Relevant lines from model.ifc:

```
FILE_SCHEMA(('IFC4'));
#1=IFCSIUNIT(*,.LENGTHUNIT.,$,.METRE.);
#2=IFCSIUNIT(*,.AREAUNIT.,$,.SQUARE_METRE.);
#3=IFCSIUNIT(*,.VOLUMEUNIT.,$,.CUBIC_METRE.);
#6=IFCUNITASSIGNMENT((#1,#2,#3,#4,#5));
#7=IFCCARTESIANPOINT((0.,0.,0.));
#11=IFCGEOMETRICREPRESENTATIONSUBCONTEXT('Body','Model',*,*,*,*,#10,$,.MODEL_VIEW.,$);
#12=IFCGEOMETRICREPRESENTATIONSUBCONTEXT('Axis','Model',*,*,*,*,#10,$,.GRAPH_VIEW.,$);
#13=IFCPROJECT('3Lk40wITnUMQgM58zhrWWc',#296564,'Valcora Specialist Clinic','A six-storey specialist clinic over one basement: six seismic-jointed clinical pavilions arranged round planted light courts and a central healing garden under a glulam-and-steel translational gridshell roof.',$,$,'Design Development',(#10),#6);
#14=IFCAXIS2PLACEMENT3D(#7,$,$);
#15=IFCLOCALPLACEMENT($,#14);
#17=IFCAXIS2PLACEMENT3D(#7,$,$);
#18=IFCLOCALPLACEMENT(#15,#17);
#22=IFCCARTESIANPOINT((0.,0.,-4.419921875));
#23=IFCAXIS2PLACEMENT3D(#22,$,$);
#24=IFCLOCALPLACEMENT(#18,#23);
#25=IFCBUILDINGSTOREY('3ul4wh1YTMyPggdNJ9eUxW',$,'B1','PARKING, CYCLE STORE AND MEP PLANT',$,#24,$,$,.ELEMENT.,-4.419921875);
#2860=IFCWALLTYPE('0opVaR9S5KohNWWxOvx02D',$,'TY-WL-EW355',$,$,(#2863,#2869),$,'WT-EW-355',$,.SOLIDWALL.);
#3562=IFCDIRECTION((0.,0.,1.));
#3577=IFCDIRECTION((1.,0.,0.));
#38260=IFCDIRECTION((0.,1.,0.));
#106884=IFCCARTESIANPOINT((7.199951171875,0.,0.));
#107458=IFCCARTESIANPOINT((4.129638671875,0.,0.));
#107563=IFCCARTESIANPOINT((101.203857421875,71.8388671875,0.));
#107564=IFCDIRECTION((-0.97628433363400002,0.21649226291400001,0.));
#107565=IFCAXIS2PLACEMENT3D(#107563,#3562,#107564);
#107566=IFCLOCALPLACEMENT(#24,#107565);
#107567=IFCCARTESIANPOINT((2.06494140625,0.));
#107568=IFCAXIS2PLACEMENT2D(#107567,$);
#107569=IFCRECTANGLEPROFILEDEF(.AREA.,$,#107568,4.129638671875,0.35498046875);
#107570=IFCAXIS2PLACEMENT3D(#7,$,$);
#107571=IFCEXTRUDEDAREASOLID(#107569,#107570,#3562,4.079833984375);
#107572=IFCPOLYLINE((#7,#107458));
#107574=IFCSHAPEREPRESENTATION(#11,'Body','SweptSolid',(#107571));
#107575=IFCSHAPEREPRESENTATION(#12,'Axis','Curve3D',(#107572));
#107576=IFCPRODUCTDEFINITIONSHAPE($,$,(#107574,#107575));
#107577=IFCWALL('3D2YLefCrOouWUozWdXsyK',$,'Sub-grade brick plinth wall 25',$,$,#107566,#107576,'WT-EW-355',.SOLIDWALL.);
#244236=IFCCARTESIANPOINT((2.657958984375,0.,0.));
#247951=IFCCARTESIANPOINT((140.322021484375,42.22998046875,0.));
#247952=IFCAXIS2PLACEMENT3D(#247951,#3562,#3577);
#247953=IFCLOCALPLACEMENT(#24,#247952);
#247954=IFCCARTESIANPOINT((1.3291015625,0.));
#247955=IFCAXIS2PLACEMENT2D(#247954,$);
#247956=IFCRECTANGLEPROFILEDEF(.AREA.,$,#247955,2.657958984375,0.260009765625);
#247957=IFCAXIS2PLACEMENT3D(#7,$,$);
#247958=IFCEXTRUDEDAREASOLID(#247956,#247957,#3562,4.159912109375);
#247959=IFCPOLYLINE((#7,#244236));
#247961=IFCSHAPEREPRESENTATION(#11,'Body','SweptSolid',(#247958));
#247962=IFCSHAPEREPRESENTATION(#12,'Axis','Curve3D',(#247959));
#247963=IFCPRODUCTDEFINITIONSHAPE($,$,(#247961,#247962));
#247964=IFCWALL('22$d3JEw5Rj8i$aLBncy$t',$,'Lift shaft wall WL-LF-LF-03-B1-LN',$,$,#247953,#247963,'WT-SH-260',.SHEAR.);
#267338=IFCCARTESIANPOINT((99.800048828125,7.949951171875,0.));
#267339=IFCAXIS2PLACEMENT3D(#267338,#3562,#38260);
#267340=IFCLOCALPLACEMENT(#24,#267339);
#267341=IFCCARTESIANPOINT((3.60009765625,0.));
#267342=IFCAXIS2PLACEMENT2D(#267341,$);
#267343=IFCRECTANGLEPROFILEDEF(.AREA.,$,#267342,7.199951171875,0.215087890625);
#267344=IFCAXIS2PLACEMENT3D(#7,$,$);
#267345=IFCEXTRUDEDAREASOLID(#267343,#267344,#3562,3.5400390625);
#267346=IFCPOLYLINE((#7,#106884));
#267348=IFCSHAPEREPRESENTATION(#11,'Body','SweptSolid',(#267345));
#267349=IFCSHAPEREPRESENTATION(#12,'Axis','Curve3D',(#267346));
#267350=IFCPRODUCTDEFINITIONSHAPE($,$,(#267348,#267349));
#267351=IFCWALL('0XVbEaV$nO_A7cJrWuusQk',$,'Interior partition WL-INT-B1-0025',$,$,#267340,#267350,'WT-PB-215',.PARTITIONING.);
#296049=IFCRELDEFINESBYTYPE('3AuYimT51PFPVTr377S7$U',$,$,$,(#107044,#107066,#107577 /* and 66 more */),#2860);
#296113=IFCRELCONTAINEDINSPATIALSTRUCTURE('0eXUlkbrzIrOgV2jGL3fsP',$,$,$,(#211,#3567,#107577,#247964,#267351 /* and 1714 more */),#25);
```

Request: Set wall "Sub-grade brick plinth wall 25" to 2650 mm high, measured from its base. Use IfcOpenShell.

```python
import ifcopenshell
import ifcopenshell.geom
import ifcopenshell.util.representation
import ifcopenshell.util.shape

model = ifcopenshell.open("model.ifc")
settings = ifcopenshell.geom.settings()


def volume(element):
    """Net volume in cubic metres, openings subtracted."""
    shape = ifcopenshell.geom.create_shape(settings, element)
    return ifcopenshell.util.shape.get_volume(shape.geometry)


wall = model.by_guid("3D2YLefCrOouWUozWdXsyK")
before = volume(wall)

body = ifcopenshell.util.representation.get_representation(wall, "Model", "Body")
solid = body.Items[0]
old_height = solid.Depth
solid.Depth = 2.65
after = volume(wall)

print(f"height {old_height:g} -> {solid.Depth:g}, volume {before:.3f} -> {after:.3f} m3")

model.write("model_v2.ifc")
```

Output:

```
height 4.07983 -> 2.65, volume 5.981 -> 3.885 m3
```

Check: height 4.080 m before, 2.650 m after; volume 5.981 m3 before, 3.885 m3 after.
